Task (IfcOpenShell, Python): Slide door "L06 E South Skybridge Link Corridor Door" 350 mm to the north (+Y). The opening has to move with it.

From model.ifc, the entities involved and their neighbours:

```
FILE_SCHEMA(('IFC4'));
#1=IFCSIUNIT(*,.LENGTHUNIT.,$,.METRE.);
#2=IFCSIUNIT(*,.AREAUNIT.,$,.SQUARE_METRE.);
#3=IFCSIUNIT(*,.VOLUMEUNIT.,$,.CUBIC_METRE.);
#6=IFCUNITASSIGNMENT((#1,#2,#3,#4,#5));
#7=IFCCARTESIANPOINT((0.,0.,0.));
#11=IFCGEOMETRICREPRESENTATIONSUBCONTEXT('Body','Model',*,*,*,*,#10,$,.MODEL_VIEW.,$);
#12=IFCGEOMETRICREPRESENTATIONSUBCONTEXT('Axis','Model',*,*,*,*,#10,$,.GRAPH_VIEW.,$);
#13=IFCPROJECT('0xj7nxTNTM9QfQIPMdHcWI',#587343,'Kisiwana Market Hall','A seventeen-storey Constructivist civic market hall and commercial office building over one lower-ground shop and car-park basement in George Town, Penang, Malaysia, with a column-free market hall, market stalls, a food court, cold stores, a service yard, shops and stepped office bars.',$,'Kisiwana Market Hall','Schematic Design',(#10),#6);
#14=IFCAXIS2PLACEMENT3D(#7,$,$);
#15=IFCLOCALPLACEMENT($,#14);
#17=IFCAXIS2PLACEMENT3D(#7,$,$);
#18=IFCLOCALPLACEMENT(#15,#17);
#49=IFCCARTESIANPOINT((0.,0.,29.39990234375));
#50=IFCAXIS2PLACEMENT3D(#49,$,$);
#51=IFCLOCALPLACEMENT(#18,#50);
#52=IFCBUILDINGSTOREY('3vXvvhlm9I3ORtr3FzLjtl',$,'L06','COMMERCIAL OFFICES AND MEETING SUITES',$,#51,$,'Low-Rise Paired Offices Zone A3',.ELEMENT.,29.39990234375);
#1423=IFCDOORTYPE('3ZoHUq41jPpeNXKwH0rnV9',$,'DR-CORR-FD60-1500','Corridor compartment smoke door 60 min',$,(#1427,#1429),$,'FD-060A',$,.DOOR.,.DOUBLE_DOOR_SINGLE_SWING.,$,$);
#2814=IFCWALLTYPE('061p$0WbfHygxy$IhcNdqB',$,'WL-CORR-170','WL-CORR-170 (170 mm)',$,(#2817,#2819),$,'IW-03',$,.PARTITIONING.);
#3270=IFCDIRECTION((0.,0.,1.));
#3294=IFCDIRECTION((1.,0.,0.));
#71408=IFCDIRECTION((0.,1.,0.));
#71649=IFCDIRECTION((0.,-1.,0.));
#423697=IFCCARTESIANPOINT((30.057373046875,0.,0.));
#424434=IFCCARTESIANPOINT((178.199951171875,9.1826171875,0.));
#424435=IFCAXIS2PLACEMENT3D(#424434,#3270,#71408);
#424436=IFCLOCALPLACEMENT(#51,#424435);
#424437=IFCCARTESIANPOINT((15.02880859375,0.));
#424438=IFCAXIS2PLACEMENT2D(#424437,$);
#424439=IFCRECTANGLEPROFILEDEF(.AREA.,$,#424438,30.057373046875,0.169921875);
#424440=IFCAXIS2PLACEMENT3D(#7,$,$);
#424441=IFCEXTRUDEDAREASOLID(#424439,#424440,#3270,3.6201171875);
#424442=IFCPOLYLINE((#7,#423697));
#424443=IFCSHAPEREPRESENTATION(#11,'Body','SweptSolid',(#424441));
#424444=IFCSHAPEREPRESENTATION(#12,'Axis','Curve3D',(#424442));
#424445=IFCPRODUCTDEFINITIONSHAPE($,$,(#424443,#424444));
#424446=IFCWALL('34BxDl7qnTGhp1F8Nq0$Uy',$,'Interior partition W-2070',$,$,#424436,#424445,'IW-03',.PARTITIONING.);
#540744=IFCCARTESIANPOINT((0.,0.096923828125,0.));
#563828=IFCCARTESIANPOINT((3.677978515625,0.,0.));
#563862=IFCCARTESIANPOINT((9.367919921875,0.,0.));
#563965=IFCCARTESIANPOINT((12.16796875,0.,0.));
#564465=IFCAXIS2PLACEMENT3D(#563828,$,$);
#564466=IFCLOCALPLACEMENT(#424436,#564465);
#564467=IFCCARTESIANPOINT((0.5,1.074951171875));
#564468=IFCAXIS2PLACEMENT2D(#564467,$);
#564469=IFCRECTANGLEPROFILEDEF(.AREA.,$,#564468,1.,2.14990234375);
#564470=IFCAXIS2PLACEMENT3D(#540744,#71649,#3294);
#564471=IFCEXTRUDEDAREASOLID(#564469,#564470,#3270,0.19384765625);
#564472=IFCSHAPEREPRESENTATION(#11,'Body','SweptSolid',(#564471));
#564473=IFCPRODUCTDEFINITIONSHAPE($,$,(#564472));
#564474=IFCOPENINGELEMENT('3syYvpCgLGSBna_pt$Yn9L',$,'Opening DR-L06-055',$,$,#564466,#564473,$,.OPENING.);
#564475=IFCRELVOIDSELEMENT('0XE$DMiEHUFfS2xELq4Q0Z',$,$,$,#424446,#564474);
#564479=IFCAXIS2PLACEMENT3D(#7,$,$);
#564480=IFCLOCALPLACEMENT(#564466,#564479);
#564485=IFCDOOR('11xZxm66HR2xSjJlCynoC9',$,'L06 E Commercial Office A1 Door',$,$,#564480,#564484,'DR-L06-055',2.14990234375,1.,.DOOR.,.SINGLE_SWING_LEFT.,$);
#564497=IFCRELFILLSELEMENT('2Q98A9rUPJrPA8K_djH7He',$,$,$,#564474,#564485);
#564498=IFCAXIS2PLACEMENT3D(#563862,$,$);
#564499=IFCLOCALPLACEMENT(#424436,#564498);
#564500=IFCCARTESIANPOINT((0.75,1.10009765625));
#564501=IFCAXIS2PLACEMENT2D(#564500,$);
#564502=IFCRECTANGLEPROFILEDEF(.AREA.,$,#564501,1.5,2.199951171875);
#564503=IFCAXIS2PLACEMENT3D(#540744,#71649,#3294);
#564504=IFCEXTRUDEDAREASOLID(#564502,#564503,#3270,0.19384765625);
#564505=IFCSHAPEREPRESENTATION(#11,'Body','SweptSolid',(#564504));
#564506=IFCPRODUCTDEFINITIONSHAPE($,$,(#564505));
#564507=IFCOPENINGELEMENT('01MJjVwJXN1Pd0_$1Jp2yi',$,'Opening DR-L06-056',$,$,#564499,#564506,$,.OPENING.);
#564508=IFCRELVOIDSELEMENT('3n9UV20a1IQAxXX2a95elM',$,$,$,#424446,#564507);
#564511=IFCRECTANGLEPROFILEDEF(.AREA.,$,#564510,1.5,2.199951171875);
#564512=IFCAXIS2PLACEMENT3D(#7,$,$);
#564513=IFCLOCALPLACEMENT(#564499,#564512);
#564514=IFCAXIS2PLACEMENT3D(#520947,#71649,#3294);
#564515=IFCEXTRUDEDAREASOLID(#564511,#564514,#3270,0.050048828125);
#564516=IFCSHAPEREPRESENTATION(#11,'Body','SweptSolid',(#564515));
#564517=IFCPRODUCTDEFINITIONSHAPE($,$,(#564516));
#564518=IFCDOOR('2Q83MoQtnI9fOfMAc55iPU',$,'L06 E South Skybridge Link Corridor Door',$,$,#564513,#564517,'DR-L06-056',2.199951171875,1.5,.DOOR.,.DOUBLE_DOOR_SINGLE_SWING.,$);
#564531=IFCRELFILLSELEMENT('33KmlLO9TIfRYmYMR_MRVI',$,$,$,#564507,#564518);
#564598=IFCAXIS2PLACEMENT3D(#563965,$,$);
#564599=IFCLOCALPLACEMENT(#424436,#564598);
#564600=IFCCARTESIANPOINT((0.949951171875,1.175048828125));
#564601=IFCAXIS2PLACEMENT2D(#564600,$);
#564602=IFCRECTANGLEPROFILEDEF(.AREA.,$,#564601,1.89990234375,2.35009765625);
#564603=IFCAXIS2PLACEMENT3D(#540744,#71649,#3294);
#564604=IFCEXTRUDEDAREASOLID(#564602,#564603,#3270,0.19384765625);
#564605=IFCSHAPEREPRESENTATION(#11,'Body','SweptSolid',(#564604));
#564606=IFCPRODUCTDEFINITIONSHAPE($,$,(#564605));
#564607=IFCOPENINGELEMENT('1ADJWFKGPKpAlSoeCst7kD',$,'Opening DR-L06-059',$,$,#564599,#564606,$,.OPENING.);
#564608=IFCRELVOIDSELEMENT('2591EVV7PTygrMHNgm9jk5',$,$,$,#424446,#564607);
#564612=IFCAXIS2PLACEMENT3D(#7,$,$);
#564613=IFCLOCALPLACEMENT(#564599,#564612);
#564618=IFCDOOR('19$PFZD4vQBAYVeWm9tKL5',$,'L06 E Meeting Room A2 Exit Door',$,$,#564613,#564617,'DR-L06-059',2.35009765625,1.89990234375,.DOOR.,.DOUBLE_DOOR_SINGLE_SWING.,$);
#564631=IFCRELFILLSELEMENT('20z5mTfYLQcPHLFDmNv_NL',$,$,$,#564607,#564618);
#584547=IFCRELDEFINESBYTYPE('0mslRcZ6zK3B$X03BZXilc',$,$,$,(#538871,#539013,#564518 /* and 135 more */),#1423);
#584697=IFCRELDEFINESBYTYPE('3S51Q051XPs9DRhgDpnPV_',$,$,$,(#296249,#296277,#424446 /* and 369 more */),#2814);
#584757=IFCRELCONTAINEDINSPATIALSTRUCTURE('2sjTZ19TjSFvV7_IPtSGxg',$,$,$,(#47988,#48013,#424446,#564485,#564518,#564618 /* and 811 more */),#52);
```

```python
import ifcopenshell
import ifcopenshell.api.geometry
import ifcopenshell.util.placement
import ifcopenshell.util.unit

model = ifcopenshell.open("model.ifc")
unit_scale = ifcopenshell.util.unit.calculate_unit_scale(model)

door = model.by_guid("2Q83MoQtnI9fOfMAc55iPU")
opening = door.FillsVoids[0].RelatingOpeningElement
wall = opening.VoidsElements[0].RelatingBuildingElement

wall_matrix = ifcopenshell.util.placement.get_local_placement(wall.ObjectPlacement)
shift = wall_matrix[:3, 0] * 0.35 / unit_scale
before = ifcopenshell.util.placement.get_local_placement(door.ObjectPlacement)[:3, 3].copy()

# The door is placed relative to its opening, so it follows when the opening moves.
matrix = ifcopenshell.util.placement.get_local_placement(opening.ObjectPlacement)
matrix[:3, 3] += shift
ifcopenshell.api.geometry.edit_object_placement(
    model, product=opening, matrix=matrix, is_si=False, should_transform_children=True
)

after = ifcopenshell.util.placement.get_local_placement(door.ObjectPlacement)[:3, 3]
print("door moved by", (after - before).round(3) + 0.0)

model.write("model_updated.ifc")
```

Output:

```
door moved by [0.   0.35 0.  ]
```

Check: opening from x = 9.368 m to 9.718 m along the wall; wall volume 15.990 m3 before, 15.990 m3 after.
